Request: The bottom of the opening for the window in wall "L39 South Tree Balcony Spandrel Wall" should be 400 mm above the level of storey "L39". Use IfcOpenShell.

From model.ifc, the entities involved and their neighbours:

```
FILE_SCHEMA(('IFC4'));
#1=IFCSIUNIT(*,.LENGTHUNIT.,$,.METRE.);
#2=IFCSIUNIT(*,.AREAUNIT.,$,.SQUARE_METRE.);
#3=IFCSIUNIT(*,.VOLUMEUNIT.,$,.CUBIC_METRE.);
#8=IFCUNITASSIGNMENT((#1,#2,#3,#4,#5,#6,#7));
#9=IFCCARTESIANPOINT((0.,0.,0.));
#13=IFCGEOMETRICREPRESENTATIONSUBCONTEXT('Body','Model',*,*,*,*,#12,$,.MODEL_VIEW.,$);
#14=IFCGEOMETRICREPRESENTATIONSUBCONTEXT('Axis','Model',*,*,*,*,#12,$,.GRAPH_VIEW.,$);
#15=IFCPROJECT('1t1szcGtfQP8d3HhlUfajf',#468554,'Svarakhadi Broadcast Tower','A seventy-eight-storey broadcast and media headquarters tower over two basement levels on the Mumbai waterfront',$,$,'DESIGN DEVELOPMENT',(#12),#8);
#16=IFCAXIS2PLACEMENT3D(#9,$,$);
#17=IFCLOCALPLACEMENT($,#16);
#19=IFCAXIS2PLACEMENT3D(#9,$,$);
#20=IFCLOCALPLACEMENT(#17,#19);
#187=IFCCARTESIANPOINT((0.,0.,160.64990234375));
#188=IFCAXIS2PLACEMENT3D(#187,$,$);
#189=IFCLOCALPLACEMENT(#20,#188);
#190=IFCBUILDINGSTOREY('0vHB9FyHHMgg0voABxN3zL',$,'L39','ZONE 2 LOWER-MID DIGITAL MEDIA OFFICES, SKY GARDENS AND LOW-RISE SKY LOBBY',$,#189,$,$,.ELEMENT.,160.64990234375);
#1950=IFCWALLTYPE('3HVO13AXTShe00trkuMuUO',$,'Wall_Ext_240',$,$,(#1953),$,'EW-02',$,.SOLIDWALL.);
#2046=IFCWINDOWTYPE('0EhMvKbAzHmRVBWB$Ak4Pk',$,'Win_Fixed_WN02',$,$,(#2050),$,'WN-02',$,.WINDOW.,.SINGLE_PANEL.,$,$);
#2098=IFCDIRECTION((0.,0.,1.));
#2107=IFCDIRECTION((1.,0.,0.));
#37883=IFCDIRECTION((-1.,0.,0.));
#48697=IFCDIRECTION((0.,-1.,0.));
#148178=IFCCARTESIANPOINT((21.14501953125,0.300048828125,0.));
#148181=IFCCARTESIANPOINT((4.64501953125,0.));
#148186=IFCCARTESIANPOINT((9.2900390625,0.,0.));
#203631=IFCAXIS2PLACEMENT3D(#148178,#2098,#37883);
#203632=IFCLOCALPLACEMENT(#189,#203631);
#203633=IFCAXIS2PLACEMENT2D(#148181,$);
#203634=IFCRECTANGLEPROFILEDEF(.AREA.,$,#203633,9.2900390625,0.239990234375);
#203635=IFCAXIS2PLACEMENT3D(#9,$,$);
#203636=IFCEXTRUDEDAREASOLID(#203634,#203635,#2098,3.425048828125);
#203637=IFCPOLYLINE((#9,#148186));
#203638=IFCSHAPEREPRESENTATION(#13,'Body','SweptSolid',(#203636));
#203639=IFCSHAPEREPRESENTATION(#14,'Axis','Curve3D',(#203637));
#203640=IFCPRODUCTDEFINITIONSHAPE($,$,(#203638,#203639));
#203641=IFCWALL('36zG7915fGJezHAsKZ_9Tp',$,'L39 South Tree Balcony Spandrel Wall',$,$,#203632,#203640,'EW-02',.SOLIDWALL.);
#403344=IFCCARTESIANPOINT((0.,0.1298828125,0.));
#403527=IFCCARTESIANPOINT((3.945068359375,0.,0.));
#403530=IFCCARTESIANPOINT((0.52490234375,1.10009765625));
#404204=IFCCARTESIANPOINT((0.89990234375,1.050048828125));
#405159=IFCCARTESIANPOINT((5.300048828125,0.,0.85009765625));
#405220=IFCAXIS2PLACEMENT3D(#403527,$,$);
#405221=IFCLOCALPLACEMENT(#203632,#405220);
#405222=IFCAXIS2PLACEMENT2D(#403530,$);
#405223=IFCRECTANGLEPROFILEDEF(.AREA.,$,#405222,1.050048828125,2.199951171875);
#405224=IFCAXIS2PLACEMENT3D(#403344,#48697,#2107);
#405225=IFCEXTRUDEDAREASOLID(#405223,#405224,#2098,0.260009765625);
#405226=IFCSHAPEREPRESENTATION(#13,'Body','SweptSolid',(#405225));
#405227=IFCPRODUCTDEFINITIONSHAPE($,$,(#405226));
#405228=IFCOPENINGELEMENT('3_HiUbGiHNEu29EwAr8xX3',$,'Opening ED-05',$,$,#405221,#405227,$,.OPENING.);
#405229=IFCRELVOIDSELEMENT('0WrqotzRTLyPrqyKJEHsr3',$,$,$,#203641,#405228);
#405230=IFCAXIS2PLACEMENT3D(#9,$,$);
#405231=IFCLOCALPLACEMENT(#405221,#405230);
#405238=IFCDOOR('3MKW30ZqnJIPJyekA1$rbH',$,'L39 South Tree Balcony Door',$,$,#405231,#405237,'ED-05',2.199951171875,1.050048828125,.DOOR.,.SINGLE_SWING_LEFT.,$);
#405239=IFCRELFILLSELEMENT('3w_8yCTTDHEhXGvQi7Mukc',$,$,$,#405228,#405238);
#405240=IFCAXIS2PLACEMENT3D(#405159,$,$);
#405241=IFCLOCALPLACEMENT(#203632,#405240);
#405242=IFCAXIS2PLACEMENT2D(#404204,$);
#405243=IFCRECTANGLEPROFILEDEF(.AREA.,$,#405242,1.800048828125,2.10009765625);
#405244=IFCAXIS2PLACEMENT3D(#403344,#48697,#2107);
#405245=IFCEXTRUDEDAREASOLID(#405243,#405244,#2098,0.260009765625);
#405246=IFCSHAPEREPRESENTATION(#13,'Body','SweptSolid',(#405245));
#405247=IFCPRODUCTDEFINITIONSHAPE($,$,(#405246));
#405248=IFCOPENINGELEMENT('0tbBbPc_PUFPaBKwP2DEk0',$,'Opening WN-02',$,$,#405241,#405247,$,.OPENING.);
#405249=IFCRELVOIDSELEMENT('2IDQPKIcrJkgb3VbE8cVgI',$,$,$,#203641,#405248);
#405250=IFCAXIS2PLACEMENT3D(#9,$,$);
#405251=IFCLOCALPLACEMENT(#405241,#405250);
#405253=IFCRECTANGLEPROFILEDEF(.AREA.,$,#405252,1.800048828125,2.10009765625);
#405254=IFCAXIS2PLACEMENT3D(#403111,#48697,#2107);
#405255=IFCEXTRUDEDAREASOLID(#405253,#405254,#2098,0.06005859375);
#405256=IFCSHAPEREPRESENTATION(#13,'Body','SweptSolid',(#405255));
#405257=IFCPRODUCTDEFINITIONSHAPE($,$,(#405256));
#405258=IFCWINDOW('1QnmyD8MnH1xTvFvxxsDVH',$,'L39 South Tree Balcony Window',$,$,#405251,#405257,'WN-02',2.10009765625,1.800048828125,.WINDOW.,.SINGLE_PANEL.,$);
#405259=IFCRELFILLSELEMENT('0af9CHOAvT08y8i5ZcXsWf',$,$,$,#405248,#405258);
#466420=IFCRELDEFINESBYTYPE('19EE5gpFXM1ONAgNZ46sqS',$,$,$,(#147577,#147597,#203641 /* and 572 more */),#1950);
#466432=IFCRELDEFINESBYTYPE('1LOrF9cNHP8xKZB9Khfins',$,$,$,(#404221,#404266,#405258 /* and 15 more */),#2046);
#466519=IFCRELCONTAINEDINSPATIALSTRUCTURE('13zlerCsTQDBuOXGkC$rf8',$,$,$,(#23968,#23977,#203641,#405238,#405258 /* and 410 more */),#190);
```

```python
import numpy as np
import ifcopenshell
import ifcopenshell.api.geometry
import ifcopenshell.geom
import ifcopenshell.util.element
import ifcopenshell.util.placement
import ifcopenshell.util.shape
import ifcopenshell.util.unit

model = ifcopenshell.open("model.ifc")
unit_scale = ifcopenshell.util.unit.calculate_unit_scale(model)

window = model.by_guid("1QnmyD8MnH1xTvFvxxsDVH")
opening = window.FillsVoids[0].RelatingOpeningElement
storey = ifcopenshell.util.element.get_container(window, ifc_class="IfcBuildingStorey")
level = ifcopenshell.util.placement.get_local_placement(storey.ObjectPlacement)[2, 3]

# The opening's origin need not be at the sill, so measure its lowest point.
shape = ifcopenshell.geom.create_shape(ifcopenshell.geom.settings(), opening)
bottom = ifcopenshell.util.shape.get_shape_bottom_elevation(shape, shape.geometry) / unit_scale
dz = level + 0.4 / unit_scale - bottom

shift = np.array([0.0, 0.0, dz])
# The window is placed relative to its opening, so it follows when the opening moves.
matrix = ifcopenshell.util.placement.get_local_placement(opening.ObjectPlacement)
matrix[:3, 3] += shift
ifcopenshell.api.geometry.edit_object_placement(
    model, product=opening, matrix=matrix, is_si=False, should_transform_children=True
)

print(f"moved by {dz * unit_scale:+.3f} m")

model.write("model_updated.ifc")
```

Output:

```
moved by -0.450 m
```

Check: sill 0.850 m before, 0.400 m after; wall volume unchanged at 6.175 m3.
